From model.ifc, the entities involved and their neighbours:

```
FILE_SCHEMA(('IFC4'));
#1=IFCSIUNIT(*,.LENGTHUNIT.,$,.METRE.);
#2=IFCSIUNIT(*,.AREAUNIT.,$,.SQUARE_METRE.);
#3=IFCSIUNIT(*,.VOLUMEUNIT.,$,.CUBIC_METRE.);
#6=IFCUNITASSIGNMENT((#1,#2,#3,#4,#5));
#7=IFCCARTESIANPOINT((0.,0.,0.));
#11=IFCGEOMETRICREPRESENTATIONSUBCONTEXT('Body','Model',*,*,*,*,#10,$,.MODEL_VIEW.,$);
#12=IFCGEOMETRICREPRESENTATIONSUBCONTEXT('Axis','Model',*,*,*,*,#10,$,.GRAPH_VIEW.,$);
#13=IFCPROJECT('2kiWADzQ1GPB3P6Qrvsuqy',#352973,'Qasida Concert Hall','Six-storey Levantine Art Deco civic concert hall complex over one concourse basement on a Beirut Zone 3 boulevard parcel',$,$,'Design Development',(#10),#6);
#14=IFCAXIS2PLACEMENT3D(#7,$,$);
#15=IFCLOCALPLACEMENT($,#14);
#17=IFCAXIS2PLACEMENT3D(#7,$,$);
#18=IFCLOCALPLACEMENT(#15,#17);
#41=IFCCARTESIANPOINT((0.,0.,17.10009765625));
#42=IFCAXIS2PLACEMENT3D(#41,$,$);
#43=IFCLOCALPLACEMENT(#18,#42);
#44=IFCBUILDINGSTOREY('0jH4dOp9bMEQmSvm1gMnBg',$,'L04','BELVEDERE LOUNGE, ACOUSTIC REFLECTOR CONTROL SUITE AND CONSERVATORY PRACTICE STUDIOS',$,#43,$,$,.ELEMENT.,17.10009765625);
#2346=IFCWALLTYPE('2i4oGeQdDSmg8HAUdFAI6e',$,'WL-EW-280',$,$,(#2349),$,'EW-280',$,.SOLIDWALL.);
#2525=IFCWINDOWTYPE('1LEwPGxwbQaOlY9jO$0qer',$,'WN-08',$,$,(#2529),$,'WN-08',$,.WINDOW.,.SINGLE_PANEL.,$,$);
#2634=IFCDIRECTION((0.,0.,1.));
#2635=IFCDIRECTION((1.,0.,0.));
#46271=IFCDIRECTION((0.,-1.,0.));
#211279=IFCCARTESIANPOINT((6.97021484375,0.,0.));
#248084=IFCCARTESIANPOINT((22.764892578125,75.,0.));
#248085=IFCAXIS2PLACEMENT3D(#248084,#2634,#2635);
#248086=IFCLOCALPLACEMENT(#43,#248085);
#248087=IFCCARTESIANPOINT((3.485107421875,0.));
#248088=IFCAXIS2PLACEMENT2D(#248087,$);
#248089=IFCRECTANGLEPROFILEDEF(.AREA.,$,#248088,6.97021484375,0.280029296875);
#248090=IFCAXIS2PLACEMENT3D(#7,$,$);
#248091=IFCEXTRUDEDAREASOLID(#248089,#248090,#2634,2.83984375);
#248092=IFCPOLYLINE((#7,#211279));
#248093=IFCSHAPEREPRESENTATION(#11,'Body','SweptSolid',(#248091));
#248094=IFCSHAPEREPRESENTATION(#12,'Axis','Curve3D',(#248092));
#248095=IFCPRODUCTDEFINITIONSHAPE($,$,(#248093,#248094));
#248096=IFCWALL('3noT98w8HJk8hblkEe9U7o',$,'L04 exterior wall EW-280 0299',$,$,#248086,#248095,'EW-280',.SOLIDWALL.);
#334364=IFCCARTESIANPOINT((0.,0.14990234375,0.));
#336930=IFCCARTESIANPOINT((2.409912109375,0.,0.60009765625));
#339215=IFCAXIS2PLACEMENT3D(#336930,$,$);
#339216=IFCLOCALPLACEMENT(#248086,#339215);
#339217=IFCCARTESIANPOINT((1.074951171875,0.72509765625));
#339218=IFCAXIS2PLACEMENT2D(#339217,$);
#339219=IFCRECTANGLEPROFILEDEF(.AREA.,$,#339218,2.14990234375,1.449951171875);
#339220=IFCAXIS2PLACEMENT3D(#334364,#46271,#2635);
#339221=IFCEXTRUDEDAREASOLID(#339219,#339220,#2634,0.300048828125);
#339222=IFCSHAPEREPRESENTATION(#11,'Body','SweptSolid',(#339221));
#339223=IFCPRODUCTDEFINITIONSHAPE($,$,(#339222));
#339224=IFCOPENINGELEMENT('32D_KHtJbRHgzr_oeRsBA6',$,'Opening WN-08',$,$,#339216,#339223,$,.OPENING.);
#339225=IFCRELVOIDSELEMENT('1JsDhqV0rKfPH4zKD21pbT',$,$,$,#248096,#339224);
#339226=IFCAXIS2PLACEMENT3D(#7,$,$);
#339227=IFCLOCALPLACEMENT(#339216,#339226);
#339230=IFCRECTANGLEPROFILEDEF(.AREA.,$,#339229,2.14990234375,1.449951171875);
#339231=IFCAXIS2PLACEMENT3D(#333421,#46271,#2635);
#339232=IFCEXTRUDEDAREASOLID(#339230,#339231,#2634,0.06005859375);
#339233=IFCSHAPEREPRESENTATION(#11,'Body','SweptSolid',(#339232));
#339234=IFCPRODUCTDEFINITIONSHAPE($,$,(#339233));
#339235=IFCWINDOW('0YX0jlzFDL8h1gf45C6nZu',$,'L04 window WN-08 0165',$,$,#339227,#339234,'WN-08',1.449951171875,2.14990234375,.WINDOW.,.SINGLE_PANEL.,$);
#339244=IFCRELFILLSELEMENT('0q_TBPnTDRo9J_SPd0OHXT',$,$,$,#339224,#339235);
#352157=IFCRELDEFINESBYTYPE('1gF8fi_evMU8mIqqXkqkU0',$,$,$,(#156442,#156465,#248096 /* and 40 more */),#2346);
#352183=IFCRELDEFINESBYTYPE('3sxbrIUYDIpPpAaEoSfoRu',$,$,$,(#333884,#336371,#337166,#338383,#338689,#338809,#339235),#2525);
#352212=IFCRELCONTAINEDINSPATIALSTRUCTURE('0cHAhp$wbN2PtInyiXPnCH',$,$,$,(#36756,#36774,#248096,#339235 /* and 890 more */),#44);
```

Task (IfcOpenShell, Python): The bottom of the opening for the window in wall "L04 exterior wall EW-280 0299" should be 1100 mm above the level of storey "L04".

```python
import numpy as np
import ifcopenshell
import ifcopenshell.api.geometry
import ifcopenshell.geom
import ifcopenshell.util.element
import ifcopenshell.util.placement
import ifcopenshell.util.shape
import ifcopenshell.util.unit

model = ifcopenshell.open("model.ifc")
unit_scale = ifcopenshell.util.unit.calculate_unit_scale(model)

window = model.by_guid("0YX0jlzFDL8h1gf45C6nZu")
opening = window.FillsVoids[0].RelatingOpeningElement
storey = ifcopenshell.util.element.get_container(window, ifc_class="IfcBuildingStorey")
level = ifcopenshell.util.placement.get_local_placement(storey.ObjectPlacement)[2, 3]

# The opening's origin need not be at the sill, so measure its lowest point.
shape = ifcopenshell.geom.create_shape(ifcopenshell.geom.settings(), opening)
bottom = ifcopenshell.util.shape.get_shape_bottom_elevation(shape, shape.geometry) / unit_scale
dz = level + 1.1 / unit_scale - bottom

shift = np.array([0.0, 0.0, dz])
# The window is placed relative to its opening, so it follows when the opening moves.
matrix = ifcopenshell.util.placement.get_local_placement(opening.ObjectPlacement)
matrix[:3, 3] += shift
ifcopenshell.api.geometry.edit_object_placement(
    model, product=opening, matrix=matrix, is_si=False, should_transform_children=True
)

print(f"moved by {dz * unit_scale:+.3f} m")

model.write("model_edited.ifc")
```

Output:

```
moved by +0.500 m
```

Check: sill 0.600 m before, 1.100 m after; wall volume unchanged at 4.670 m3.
